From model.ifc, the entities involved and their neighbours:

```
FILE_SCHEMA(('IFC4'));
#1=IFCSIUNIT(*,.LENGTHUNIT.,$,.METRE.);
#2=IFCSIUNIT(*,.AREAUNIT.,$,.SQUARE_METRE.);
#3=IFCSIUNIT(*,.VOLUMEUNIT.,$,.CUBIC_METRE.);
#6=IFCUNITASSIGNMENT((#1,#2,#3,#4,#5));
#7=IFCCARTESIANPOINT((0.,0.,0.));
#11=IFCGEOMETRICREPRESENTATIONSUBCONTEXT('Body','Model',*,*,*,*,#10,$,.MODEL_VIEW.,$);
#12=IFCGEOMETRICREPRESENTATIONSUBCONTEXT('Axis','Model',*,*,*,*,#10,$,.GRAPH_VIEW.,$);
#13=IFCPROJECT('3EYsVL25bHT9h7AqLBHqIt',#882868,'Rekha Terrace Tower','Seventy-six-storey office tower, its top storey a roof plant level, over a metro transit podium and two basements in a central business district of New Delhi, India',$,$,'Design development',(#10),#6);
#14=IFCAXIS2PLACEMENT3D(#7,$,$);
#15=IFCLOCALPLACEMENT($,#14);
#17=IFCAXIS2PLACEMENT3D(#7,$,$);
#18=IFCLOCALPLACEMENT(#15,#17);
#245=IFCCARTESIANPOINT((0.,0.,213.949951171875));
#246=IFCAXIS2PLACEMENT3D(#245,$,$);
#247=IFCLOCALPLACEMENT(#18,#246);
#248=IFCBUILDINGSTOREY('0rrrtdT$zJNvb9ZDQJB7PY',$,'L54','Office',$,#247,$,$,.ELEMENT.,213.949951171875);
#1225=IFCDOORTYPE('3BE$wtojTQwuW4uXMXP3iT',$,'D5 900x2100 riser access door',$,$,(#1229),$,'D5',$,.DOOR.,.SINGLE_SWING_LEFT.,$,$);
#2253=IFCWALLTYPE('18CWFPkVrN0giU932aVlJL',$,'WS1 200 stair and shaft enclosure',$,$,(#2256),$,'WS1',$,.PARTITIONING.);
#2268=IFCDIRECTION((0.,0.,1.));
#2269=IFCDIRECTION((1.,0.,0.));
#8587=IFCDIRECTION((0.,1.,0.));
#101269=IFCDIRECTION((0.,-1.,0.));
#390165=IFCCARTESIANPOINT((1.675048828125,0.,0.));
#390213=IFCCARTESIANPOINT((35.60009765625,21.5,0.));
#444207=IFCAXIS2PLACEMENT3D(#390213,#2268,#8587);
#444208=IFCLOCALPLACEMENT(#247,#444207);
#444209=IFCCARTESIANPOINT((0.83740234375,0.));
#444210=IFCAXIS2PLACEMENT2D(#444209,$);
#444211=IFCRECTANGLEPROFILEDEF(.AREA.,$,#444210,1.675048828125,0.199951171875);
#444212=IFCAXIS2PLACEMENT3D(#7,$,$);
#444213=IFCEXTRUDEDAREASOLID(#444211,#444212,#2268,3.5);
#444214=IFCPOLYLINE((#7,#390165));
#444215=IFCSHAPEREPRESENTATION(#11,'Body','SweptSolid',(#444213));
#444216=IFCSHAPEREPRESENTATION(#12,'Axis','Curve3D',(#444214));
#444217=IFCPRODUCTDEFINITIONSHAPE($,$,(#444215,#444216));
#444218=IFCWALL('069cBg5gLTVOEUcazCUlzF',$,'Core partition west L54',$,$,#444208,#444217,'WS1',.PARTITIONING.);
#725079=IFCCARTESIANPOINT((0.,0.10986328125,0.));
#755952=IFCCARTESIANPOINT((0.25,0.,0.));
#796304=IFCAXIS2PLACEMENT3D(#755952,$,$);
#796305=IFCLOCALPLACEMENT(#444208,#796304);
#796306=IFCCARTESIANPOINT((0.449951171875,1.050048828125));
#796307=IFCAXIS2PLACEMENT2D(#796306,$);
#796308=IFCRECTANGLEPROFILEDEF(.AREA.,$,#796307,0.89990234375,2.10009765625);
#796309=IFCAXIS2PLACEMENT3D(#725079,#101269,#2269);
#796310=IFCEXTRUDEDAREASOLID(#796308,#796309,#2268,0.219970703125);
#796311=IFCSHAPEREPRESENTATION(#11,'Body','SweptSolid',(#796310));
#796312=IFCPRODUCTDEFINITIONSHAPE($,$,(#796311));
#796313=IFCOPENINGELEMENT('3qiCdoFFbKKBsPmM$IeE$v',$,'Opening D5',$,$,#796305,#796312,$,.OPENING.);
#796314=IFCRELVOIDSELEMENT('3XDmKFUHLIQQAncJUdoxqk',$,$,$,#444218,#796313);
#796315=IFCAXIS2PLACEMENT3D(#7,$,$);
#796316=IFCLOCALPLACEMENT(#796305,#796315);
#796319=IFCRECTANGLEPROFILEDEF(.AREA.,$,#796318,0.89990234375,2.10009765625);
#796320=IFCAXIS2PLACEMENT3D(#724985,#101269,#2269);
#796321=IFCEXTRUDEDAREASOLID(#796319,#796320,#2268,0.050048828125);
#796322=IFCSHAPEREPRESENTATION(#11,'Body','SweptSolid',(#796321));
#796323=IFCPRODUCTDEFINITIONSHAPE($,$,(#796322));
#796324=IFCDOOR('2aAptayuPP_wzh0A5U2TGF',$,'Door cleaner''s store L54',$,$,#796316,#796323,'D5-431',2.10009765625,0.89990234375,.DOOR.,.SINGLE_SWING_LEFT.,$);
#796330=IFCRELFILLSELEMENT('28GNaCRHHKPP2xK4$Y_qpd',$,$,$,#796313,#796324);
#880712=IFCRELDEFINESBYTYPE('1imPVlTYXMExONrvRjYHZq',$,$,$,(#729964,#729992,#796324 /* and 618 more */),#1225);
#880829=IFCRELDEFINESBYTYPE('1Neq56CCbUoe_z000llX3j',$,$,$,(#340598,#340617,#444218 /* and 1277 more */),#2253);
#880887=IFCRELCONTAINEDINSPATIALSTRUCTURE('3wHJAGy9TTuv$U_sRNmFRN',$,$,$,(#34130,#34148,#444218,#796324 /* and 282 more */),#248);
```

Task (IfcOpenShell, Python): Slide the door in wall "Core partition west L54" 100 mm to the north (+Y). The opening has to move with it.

```python
import ifcopenshell
import ifcopenshell.api.geometry
import ifcopenshell.util.placement
import ifcopenshell.util.unit

model = ifcopenshell.open("model.ifc")
unit_scale = ifcopenshell.util.unit.calculate_unit_scale(model)

door = model.by_guid("2aAptayuPP_wzh0A5U2TGF")
opening = door.FillsVoids[0].RelatingOpeningElement
wall = opening.VoidsElements[0].RelatingBuildingElement

wall_matrix = ifcopenshell.util.placement.get_local_placement(wall.ObjectPlacement)
shift = wall_matrix[:3, 0] * 0.1 / unit_scale
before = ifcopenshell.util.placement.get_local_placement(door.ObjectPlacement)[:3, 3].copy()

# The door is placed relative to its opening, so it follows when the opening moves.
matrix = ifcopenshell.util.placement.get_local_placement(opening.ObjectPlacement)
matrix[:3, 3] += shift
ifcopenshell.api.geometry.edit_object_placement(
    model, product=opening, matrix=matrix, is_si=False, should_transform_children=True
)

after = ifcopenshell.util.placement.get_local_placement(door.ObjectPlacement)[:3, 3]
print("door moved by", (after - before).round(3) + 0.0)

model.write("model-out.ifc")
```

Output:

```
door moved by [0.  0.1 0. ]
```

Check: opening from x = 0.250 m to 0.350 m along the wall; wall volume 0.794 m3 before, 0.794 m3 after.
